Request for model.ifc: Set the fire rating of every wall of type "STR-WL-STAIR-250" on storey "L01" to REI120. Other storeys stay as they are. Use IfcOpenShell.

First a look at what the model holds.

```python
import ifcopenshell
import ifcopenshell.util.element

model = ifcopenshell.open("model.ifc")
print(model.schema)
storey = next(s for s in model.by_type("IfcBuildingStorey") if s.Name == "L01")
walls = [e for e in ifcopenshell.util.element.get_decomposition(storey) if e.is_a("IfcWall")]
seen = {}
for e in walls:
    element_type = ifcopenshell.util.element.get_type(e)
    key = (element_type.Name if element_type != e and element_type else None, ifcopenshell.util.element.get_pset(e, "Pset_WallCommon", "FireRating"))
    seen[key] = seen.get(key, 0) + 1
for (name, value), count in sorted(seen.items(), key=str):
    print(count, "x", name, "|", value)
```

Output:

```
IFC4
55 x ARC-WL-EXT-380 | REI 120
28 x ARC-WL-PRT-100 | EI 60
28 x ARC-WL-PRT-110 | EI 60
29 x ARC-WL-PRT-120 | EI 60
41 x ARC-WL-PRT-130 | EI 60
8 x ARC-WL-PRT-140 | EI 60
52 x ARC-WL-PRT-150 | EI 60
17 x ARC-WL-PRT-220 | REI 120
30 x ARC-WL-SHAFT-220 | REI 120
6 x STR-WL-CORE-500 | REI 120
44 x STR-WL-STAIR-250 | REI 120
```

```python
import ifcopenshell
import ifcopenshell.api.pset
import ifcopenshell.util.element

model = ifcopenshell.open("model.ifc")

storey = next(s for s in model.by_type("IfcBuildingStorey") if s.Name == "L01")
walls = [e for e in ifcopenshell.util.element.get_decomposition(storey) if e.is_a("IfcWall")]

count = 0
for e in walls:
    element_type = ifcopenshell.util.element.get_type(e)
    if element_type in (None, e) or element_type.Name != "STR-WL-STAIR-250":
        continue
    # add_pset returns the element's existing set when there is one.
    pset = ifcopenshell.api.pset.add_pset(model, product=e, name="Pset_WallCommon")
    ifcopenshell.api.pset.edit_pset(model, pset=pset, properties={"FireRating": "REI120"})
    count += 1

print(count, "walls updated")

model.write("model_updated.ifc")
```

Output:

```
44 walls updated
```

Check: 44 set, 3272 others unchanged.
